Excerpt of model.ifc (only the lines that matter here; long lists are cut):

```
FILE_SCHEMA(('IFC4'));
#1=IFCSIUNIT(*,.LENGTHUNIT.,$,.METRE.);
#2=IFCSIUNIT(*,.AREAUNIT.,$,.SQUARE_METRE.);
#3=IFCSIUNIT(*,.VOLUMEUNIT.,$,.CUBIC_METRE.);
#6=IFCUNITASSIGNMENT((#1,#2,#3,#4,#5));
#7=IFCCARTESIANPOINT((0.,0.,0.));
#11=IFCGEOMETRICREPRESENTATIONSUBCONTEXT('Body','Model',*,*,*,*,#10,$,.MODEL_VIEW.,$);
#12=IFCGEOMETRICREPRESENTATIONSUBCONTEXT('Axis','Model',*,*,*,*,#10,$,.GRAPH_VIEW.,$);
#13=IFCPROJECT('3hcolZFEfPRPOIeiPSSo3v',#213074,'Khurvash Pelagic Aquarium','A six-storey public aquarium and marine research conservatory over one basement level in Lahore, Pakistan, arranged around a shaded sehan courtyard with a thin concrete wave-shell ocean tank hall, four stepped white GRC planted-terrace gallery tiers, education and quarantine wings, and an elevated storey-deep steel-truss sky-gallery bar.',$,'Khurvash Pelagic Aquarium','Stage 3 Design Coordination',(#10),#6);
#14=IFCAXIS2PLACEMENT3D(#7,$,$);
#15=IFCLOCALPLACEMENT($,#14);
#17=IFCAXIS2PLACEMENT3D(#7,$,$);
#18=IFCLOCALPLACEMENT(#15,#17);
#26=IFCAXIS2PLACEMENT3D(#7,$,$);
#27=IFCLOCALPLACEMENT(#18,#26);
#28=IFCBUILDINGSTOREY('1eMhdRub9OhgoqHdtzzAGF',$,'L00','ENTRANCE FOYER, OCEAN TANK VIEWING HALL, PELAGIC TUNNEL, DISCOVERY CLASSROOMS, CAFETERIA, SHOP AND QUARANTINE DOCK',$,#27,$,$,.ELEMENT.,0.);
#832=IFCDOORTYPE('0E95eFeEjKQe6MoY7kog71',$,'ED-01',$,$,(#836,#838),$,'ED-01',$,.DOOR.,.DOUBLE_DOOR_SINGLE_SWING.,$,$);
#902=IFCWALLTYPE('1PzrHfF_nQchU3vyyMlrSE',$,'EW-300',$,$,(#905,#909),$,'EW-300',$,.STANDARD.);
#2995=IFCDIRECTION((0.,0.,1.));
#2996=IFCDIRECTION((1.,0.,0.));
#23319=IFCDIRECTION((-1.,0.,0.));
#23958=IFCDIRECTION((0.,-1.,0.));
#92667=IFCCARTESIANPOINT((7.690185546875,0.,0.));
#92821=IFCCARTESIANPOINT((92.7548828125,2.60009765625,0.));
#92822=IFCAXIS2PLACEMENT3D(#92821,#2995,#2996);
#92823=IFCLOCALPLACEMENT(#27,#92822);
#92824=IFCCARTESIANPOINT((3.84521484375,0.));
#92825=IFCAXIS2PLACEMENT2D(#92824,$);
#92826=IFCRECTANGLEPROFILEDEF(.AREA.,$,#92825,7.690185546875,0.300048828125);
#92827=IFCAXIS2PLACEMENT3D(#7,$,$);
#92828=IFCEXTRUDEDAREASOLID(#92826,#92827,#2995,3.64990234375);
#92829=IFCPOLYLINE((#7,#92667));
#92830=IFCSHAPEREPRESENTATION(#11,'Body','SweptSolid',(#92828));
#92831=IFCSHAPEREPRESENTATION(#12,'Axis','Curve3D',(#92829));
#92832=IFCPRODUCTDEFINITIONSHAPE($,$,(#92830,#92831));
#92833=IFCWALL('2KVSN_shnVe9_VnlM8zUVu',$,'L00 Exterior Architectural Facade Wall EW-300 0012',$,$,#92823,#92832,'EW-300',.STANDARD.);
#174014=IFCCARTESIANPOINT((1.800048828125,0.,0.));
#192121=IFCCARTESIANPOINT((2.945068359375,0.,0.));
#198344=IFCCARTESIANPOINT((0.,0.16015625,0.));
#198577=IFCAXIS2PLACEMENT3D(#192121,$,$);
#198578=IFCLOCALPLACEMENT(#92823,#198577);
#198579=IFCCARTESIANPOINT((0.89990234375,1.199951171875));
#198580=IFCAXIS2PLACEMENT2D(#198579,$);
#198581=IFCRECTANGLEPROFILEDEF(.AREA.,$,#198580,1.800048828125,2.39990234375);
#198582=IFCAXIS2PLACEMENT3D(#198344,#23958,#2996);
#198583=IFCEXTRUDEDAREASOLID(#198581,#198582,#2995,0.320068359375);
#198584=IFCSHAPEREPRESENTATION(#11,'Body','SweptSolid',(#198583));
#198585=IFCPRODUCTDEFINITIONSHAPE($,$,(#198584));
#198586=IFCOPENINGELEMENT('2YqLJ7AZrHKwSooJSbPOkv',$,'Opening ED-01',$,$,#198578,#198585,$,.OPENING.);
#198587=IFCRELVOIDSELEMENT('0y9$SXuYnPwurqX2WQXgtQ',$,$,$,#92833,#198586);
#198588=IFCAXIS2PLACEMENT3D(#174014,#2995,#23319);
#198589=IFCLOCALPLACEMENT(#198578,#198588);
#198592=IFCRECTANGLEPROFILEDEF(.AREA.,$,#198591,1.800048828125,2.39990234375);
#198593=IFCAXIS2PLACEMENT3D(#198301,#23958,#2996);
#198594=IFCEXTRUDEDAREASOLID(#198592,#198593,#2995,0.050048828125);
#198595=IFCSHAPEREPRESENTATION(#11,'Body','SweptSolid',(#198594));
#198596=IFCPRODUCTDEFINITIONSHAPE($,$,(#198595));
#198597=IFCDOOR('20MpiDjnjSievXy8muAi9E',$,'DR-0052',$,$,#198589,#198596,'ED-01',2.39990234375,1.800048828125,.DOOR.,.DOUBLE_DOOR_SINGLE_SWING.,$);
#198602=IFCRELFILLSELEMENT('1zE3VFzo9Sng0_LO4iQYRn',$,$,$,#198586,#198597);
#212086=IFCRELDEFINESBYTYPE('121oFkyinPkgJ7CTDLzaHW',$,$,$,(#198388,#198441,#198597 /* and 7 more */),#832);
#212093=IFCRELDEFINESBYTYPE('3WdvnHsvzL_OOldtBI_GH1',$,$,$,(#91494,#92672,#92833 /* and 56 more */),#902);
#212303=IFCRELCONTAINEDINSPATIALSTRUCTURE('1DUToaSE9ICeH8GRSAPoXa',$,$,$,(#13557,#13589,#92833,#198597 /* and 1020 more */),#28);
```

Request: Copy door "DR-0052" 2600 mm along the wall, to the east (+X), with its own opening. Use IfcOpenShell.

```python
import ifcopenshell
import ifcopenshell.api.feature
import ifcopenshell.api.geometry
import ifcopenshell.api.root
import ifcopenshell.geom
import ifcopenshell.util.element
import ifcopenshell.util.placement
import ifcopenshell.util.shape
import ifcopenshell.util.unit

model = ifcopenshell.open("model.ifc")
unit_scale = ifcopenshell.util.unit.calculate_unit_scale(model)
settings = ifcopenshell.geom.settings()


def volume(element):
    """Net volume in cubic metres, openings subtracted."""
    shape = ifcopenshell.geom.create_shape(settings, element)
    return ifcopenshell.util.shape.get_volume(shape.geometry)


door = model.by_guid("20MpiDjnjSievXy8muAi9E")
opening = door.FillsVoids[0].RelatingOpeningElement
wall = opening.VoidsElements[0].RelatingBuildingElement
before = volume(wall)
shift = ifcopenshell.util.placement.get_local_placement(wall.ObjectPlacement)[:3, 0] * 2.6 / unit_scale

# copy_class copies the void relationship, type, container and properties, but no geometry.
new_opening = ifcopenshell.api.root.copy_class(model, product=opening)
new_opening.Representation = ifcopenshell.util.element.copy_deep(
    model, opening.Representation, exclude=["IfcGeometricRepresentationContext", "IfcRepresentationMap"]
)
new_door = ifcopenshell.api.root.copy_class(model, product=door)
new_door.Representation = ifcopenshell.util.element.copy_deep(
    model, door.Representation, exclude=["IfcGeometricRepresentationContext", "IfcRepresentationMap"]
)
new_door.Tag = None
ifcopenshell.api.feature.add_filling(model, opening=new_opening, element=new_door)

for old, new in ((opening, new_opening), (door, new_door)):
    matrix = ifcopenshell.util.placement.get_local_placement(old.ObjectPlacement)
    matrix[:3, 3] += shift
    ifcopenshell.api.geometry.edit_object_placement(model, product=new, matrix=matrix, is_si=False)

after = volume(wall)

print(f"wall volume {before:.3f} -> {after:.3f} m3")

model.write("model_v2.ifc")
```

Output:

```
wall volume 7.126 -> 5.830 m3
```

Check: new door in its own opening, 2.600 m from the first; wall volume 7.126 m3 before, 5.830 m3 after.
